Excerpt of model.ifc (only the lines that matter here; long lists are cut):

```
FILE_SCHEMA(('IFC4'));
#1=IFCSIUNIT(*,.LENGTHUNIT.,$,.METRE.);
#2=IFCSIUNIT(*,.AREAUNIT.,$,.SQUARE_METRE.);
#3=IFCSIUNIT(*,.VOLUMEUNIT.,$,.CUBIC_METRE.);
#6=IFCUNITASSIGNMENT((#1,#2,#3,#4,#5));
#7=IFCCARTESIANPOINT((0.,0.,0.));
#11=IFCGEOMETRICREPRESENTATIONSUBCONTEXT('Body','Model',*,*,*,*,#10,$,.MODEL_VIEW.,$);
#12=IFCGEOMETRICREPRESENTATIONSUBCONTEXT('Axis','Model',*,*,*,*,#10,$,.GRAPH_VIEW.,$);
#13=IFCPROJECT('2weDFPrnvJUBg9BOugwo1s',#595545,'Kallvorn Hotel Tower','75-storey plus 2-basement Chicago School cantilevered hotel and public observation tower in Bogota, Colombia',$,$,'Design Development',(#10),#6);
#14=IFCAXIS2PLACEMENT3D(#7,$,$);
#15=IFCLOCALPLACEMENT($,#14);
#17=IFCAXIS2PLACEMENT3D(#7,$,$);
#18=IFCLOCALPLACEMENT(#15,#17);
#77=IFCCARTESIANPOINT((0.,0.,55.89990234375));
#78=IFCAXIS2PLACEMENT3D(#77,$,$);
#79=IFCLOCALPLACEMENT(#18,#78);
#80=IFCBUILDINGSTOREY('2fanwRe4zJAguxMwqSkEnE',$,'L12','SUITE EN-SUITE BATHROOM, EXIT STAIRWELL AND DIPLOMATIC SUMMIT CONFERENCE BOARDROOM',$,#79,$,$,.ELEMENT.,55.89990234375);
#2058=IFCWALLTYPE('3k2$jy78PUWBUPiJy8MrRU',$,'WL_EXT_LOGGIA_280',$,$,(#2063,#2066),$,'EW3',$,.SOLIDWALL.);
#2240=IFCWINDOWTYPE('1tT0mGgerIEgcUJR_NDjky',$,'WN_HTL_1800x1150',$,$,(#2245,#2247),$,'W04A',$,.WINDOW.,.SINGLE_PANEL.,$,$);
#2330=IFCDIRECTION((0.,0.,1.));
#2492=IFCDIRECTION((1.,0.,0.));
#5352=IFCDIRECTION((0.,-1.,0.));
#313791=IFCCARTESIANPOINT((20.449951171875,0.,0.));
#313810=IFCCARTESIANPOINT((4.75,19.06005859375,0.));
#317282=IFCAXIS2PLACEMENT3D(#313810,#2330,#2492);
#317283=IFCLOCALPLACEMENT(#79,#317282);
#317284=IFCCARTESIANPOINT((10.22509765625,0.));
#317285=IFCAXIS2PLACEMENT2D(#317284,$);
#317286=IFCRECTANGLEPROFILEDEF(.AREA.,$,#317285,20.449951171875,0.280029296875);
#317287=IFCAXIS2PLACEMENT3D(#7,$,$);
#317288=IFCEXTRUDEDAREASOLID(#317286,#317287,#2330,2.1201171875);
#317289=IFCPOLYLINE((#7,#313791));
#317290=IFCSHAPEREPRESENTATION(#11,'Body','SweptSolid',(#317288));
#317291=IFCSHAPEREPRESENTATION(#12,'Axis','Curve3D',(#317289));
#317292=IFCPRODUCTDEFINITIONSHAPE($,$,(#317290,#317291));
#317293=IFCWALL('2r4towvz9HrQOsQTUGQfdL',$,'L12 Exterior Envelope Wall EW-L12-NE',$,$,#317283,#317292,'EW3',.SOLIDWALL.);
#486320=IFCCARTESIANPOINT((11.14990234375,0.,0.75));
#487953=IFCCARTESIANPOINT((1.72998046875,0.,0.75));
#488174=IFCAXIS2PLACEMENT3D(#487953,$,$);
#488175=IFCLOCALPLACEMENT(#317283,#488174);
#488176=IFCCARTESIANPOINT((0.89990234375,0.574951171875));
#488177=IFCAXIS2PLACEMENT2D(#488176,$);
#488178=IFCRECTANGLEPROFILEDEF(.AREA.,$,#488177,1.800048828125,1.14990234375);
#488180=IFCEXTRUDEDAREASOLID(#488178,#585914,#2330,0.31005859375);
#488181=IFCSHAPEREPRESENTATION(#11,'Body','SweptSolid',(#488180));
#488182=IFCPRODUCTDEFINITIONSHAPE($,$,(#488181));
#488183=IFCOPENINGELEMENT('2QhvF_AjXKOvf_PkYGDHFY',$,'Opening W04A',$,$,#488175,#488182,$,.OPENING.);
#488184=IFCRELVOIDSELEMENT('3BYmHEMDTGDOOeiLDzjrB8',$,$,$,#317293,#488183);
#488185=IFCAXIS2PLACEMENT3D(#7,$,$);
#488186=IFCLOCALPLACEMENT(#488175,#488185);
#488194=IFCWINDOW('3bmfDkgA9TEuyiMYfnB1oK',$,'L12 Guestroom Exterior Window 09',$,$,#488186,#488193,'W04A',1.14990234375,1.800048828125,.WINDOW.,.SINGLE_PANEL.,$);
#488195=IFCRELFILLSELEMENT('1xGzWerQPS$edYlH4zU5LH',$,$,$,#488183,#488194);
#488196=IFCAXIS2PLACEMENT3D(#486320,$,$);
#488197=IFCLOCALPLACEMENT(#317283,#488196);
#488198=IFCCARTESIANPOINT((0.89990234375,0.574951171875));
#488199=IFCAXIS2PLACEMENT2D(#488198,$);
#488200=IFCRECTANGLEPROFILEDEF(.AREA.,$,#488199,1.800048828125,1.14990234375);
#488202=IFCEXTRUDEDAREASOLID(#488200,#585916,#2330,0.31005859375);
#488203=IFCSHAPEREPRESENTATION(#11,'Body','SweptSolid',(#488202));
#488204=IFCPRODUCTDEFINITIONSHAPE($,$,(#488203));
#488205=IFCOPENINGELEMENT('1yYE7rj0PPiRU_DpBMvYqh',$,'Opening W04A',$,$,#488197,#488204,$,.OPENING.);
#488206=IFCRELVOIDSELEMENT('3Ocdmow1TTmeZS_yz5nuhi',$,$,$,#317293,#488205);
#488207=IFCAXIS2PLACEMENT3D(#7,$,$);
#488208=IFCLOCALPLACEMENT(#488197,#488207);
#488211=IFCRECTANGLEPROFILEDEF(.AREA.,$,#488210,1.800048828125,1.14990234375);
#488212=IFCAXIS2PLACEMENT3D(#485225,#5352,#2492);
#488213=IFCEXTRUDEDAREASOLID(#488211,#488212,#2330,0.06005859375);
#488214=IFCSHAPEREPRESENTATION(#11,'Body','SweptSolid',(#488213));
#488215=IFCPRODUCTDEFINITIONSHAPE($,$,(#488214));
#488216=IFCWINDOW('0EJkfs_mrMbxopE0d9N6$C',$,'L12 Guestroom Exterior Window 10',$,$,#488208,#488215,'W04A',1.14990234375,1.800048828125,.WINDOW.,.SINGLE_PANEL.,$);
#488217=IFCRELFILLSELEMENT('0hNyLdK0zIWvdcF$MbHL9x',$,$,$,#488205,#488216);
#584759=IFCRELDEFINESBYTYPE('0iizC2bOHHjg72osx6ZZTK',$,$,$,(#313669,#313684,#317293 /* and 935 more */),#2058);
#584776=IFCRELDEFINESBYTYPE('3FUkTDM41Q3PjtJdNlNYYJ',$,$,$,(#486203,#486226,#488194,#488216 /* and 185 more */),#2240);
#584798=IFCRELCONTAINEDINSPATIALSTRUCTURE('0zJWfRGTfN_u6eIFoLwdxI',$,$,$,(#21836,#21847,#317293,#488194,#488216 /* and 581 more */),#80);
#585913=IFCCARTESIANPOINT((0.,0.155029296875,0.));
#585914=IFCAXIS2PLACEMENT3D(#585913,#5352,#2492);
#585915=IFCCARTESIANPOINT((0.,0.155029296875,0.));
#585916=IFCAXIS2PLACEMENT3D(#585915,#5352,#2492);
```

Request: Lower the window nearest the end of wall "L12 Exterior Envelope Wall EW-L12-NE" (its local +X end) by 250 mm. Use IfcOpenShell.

```python
import numpy as np
import ifcopenshell
import ifcopenshell.api.geometry
import ifcopenshell.util.placement
import ifcopenshell.util.unit

model = ifcopenshell.open("model.ifc")
unit_scale = ifcopenshell.util.unit.calculate_unit_scale(model)

window = model.by_guid("0EJkfs_mrMbxopE0d9N6$C")
opening = window.FillsVoids[0].RelatingOpeningElement
dz = -0.25

shift = np.array([0.0, 0.0, dz])
# The window is placed relative to its opening, so it follows when the opening moves.
matrix = ifcopenshell.util.placement.get_local_placement(opening.ObjectPlacement)
matrix[:3, 3] += shift
ifcopenshell.api.geometry.edit_object_placement(
    model, product=opening, matrix=matrix, is_si=False, should_transform_children=True
)

print(f"moved by {dz * unit_scale:+.3f} m")

model.write("model_updated.ifc")
```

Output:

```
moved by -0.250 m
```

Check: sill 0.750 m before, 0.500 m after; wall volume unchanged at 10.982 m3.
